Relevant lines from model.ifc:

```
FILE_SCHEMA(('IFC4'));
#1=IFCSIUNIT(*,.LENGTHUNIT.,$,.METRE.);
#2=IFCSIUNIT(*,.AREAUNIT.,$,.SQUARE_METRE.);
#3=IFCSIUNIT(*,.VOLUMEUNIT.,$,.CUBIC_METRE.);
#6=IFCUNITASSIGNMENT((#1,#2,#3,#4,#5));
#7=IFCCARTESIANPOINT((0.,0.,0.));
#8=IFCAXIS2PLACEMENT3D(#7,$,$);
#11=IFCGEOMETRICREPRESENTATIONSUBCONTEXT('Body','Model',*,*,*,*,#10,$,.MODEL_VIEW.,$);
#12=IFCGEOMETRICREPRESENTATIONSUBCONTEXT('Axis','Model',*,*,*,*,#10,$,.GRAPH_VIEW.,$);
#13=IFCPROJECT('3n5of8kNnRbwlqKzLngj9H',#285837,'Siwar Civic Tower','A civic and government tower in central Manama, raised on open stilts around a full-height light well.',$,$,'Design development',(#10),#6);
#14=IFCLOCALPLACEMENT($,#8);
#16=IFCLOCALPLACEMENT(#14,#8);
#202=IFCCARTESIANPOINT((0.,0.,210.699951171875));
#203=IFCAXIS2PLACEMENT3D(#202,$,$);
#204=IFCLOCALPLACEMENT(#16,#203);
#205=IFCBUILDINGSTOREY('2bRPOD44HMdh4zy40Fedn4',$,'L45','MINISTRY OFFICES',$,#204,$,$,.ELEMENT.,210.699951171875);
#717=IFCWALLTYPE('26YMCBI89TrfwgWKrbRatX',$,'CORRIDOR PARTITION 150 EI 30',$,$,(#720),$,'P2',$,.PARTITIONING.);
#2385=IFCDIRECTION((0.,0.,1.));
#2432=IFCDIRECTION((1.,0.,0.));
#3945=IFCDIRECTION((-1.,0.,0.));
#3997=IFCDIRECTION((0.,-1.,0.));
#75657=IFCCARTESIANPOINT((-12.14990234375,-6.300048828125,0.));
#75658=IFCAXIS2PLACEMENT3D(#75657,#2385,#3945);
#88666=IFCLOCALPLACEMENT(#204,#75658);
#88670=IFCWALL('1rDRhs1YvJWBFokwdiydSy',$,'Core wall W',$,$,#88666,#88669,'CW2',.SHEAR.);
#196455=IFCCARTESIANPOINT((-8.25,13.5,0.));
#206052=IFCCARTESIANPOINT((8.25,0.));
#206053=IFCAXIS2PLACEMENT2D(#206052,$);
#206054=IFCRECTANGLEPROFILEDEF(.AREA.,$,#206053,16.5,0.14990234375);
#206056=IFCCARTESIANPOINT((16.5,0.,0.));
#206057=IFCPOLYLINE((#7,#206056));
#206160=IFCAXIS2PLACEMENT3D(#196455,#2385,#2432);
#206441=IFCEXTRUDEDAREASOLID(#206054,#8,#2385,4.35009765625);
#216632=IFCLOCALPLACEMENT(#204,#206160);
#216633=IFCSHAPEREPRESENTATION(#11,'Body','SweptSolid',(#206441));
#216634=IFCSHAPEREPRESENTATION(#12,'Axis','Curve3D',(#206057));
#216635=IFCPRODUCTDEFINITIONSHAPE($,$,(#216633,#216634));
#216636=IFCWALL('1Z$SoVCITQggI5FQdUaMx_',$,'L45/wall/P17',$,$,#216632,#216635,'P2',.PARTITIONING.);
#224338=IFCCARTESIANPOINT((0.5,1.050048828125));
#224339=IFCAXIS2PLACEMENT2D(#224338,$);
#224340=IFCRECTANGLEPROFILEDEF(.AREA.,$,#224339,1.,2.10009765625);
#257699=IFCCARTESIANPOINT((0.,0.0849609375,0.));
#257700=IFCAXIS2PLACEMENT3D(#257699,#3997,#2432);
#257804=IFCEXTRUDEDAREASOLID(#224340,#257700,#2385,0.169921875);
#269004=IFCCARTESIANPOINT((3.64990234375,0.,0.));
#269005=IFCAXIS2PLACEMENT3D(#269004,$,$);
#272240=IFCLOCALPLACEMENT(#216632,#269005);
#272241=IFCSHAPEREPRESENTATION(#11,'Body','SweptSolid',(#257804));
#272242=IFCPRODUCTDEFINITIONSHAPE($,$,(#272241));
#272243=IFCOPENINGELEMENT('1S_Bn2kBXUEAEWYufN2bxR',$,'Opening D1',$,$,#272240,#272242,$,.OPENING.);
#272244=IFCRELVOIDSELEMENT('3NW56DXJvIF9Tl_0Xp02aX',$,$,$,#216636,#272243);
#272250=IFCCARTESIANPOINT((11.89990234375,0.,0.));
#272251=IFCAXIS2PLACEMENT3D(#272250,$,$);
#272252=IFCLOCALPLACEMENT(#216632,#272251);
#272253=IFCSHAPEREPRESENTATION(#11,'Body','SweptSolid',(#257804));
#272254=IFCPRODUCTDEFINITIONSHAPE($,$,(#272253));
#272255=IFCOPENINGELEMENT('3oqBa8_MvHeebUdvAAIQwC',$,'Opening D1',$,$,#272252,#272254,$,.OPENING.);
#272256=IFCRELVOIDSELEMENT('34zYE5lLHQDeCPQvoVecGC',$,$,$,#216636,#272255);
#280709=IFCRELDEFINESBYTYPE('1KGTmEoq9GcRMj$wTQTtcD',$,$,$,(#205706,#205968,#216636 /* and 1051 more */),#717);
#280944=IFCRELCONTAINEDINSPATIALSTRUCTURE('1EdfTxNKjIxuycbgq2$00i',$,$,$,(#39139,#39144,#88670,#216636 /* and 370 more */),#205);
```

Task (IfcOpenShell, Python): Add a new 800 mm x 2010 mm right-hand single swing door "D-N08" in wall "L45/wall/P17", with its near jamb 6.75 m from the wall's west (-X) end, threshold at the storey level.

```python
import numpy as np
import ifcopenshell
import ifcopenshell.api.feature
import ifcopenshell.api.geometry
import ifcopenshell.api.root
import ifcopenshell.api.spatial
import ifcopenshell.geom
import ifcopenshell.util.element
import ifcopenshell.util.placement
import ifcopenshell.util.representation
import ifcopenshell.util.shape
import ifcopenshell.util.unit

model = ifcopenshell.open("model.ifc")
unit_scale = ifcopenshell.util.unit.calculate_unit_scale(model)
settings = ifcopenshell.geom.settings()


def volume(element):
    """Net volume in cubic metres, openings subtracted."""
    shape = ifcopenshell.geom.create_shape(settings, element)
    return ifcopenshell.util.shape.get_volume(shape.geometry)


wall = model.by_guid("1Z$SoVCITQggI5FQdUaMx_")
storey = ifcopenshell.util.element.get_container(wall, ifc_class="IfcBuildingStorey")
context = ifcopenshell.util.representation.get_context(model, "Model", "Body", "MODEL_VIEW")
before = volume(wall)

width, height, from_end, sill = 0.8, 2.01, 6.75, 0.0  # metres

# The wall runs along its own X axis, and the end named is its -X end.
wall_shape = ifcopenshell.geom.create_shape(settings, wall)
x, y, z = ifcopenshell.util.shape.get_vertices(wall_shape.geometry).T
start = x.min() + from_end
face, thickness = float(y.min()), float(y.max() - y.min())
wall_matrix = ifcopenshell.util.placement.get_local_placement(wall.ObjectPlacement)
level = ifcopenshell.util.placement.get_local_placement(storey.ObjectPlacement)[2, 3]


def in_wall(x, y):
    """Placement at x, y metres in the wall's axes, at sill height."""
    matrix = wall_matrix.copy()
    matrix[:, 3] = wall_matrix @ np.array([x / unit_scale, y / unit_scale, 0.0, 1.0])
    matrix[2, 3] = level + sill / unit_scale
    return matrix


# Opening: a box that overshoots both wall faces by 50 mm.
opening = ifcopenshell.api.root.create_entity(model, ifc_class="IfcOpeningElement", predefined_type="OPENING")
box = ifcopenshell.api.geometry.add_wall_representation(
    model, context=context, length=width, height=height, thickness=thickness + 0.1
)
ifcopenshell.api.geometry.assign_representation(model, product=opening, representation=box)
ifcopenshell.api.geometry.edit_object_placement(model, product=opening, matrix=in_wall(start, face - 0.05), is_si=False)
ifcopenshell.api.feature.add_feature(model, feature=opening, element=wall)

door = ifcopenshell.api.root.create_entity(model, ifc_class="IfcDoor", name="D-N08", predefined_type="DOOR")
door.OverallWidth, door.OverallHeight = width / unit_scale, height / unit_scale
door.OperationType = "SINGLE_SWING_RIGHT"
body = ifcopenshell.api.geometry.add_door_representation(
    model,
    context=context,
    overall_width=door.OverallWidth,
    overall_height=door.OverallHeight,
    operation_type="SINGLE_SWING_RIGHT",
    lining_properties={"LiningDepth": thickness / unit_scale, "ThresholdDepth": thickness / unit_scale},
)
ifcopenshell.api.geometry.assign_representation(model, product=door, representation=body)
ifcopenshell.api.spatial.assign_container(model, products=[door], relating_structure=storey)
ifcopenshell.api.feature.add_filling(model, opening=opening, element=door)

# The lining spans the wall, so the door starts at the wall face.
ifcopenshell.api.geometry.edit_object_placement(model, product=door, matrix=in_wall(start, face), is_si=False)

after = volume(wall)

print(f"wall volume {before:.3f} -> {after:.3f} m3")

model.write("model_v2.ifc")
```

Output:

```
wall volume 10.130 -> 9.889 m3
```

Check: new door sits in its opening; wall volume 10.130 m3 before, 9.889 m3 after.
